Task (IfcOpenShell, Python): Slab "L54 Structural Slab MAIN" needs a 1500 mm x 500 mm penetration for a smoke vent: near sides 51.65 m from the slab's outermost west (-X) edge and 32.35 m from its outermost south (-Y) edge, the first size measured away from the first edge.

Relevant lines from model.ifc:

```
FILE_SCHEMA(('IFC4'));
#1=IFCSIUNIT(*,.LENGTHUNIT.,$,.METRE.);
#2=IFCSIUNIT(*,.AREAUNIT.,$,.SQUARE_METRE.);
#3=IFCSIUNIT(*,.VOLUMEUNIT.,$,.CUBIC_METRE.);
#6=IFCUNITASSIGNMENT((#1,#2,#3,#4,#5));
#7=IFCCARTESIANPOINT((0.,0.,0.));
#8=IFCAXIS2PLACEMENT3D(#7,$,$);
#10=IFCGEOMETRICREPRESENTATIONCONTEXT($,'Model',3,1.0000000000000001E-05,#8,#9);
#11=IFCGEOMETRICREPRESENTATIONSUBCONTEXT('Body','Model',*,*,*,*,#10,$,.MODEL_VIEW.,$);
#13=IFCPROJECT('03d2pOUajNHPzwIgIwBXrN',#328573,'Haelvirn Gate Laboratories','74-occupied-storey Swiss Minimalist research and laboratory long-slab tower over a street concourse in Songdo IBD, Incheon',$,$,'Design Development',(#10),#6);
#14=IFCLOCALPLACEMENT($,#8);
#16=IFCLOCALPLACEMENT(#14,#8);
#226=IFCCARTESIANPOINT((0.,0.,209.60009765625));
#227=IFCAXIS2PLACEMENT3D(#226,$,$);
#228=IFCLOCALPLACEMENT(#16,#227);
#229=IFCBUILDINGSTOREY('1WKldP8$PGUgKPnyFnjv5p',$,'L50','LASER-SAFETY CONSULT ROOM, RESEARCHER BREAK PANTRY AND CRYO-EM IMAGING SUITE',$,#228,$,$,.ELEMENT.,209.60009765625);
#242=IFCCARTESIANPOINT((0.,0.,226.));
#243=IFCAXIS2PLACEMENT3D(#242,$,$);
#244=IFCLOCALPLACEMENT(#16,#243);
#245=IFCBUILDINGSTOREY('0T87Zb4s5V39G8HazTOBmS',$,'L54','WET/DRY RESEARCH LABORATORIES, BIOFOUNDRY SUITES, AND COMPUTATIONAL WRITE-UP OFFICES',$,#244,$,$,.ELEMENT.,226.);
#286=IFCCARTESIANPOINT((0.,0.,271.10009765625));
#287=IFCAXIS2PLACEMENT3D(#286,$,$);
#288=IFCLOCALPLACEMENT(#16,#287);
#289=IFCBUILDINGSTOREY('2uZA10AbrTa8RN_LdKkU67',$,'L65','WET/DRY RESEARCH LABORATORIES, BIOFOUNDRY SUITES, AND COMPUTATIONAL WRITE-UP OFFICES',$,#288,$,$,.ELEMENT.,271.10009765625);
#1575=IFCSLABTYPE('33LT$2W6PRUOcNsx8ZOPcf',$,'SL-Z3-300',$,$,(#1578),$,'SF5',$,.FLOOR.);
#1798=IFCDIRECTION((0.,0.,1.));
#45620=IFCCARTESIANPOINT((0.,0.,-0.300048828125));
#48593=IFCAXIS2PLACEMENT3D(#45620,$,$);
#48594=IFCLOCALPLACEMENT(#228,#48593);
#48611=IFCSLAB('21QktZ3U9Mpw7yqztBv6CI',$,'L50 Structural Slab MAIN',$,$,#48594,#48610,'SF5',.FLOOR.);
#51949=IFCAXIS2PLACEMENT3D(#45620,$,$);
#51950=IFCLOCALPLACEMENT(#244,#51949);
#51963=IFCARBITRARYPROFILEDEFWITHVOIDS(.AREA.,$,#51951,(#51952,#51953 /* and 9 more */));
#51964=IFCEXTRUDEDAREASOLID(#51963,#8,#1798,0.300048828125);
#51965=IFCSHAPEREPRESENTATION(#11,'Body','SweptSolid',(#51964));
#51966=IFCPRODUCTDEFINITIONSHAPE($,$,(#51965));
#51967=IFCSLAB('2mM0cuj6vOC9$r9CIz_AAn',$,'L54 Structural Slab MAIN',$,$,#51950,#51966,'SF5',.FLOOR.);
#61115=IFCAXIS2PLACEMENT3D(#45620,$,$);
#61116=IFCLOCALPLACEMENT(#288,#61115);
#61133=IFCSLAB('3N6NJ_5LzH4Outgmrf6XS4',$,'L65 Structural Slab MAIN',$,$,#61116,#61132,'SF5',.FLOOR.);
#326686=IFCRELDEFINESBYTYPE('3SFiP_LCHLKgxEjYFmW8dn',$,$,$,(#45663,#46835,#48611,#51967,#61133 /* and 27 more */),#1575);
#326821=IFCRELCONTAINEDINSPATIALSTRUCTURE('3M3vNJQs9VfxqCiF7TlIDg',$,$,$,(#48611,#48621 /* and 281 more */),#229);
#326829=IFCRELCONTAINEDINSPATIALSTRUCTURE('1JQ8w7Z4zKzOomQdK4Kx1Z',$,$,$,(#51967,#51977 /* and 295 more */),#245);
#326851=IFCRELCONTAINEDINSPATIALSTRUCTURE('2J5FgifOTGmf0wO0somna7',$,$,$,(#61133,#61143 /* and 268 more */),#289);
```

```python
import numpy as np
import ifcopenshell
import ifcopenshell.api.feature
import ifcopenshell.api.geometry
import ifcopenshell.api.root
import ifcopenshell.geom
import ifcopenshell.util.placement
import ifcopenshell.util.representation
import ifcopenshell.util.shape
import ifcopenshell.util.unit

model = ifcopenshell.open("model.ifc")
unit_scale = ifcopenshell.util.unit.calculate_unit_scale(model)
settings = ifcopenshell.geom.settings()


def volume(element):
    """Net volume in cubic metres, openings subtracted."""
    shape = ifcopenshell.geom.create_shape(settings, element)
    return ifcopenshell.util.shape.get_volume(shape.geometry)


slab = model.by_id(51967)
before = volume(slab)

# Extent in the slab's own axes, in metres. The edges named are its -X and -Y sides.
slab_shape = ifcopenshell.geom.create_shape(settings, slab)
vertices = ifcopenshell.util.shape.get_vertices(slab_shape.geometry)
x_min, y_min, bottom = vertices.min(axis=0)
top = vertices[:, 2].max()

opening = ifcopenshell.api.root.create_entity(model, ifc_class="IfcOpeningElement", name="Smoke vent opening", predefined_type="OPENING")
context = ifcopenshell.util.representation.get_context(model, "Model", "Body", "MODEL_VIEW")
width, depth = 1.5, 0.5
outline = [(0.0, 0.0), (width, 0.0), (width, depth), (0.0, depth), (0.0, 0.0)]
# Overshoot both faces by 50 mm so the cut is clean.
shape = ifcopenshell.api.geometry.add_slab_representation(
    model, context=context, depth=top - bottom + 0.1, polyline=outline
)
ifcopenshell.api.geometry.assign_representation(model, product=opening, representation=shape)

matrix = ifcopenshell.util.placement.get_local_placement(slab.ObjectPlacement)
matrix[:, 3] = matrix @ np.append(np.array([x_min + 51.65, y_min + 32.35, bottom - 0.05]) / unit_scale, 1.0)
ifcopenshell.api.geometry.edit_object_placement(model, product=opening, matrix=matrix, is_si=False)
ifcopenshell.api.feature.add_feature(model, feature=opening, element=slab)

after = volume(slab)

print(f"slab volume {before:.3f} -> {after:.3f} m3")

model.write("model_v2.ifc")
```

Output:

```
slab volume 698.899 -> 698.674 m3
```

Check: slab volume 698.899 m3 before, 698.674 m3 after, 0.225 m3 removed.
